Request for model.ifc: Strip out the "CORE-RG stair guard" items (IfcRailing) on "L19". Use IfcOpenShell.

First a look at what the model holds.

```python
import ifcopenshell
import ifcopenshell.util.element

model = ifcopenshell.open("model.ifc")
print(model.schema)
storey = next(s for s in model.by_type("IfcBuildingStorey") if s.Name == "L19")
railings = [e for e in ifcopenshell.util.element.get_decomposition(storey) if e.is_a("IfcRailing")]
seen = {}
for e in railings:
    element_type = ifcopenshell.util.element.get_type(e)
    name = element_type.Name if element_type not in (None, e) else None
    seen[name] = seen.get(name, 0) + 1
for name, count in sorted(seen.items(), key=str):
    print(count, "x", name)
```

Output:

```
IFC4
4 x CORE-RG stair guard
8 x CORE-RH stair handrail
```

```python
import ifcopenshell
import ifcopenshell.api.root
import ifcopenshell.util.element

model = ifcopenshell.open("model.ifc")

storey = next(s for s in model.by_type("IfcBuildingStorey") if s.Name == "L19")
railings = [e for e in ifcopenshell.util.element.get_decomposition(storey) if e.is_a("IfcRailing")]
targets = [e for e in railings if (t := ifcopenshell.util.element.get_type(e)) not in (None, e) and t.Name == "CORE-RG stair guard"]

for e in targets:
    ifcopenshell.api.root.remove_product(model, product=e)
print(len(targets), "removed")

model.write("model_rev.ifc")
```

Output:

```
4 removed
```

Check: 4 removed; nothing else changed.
